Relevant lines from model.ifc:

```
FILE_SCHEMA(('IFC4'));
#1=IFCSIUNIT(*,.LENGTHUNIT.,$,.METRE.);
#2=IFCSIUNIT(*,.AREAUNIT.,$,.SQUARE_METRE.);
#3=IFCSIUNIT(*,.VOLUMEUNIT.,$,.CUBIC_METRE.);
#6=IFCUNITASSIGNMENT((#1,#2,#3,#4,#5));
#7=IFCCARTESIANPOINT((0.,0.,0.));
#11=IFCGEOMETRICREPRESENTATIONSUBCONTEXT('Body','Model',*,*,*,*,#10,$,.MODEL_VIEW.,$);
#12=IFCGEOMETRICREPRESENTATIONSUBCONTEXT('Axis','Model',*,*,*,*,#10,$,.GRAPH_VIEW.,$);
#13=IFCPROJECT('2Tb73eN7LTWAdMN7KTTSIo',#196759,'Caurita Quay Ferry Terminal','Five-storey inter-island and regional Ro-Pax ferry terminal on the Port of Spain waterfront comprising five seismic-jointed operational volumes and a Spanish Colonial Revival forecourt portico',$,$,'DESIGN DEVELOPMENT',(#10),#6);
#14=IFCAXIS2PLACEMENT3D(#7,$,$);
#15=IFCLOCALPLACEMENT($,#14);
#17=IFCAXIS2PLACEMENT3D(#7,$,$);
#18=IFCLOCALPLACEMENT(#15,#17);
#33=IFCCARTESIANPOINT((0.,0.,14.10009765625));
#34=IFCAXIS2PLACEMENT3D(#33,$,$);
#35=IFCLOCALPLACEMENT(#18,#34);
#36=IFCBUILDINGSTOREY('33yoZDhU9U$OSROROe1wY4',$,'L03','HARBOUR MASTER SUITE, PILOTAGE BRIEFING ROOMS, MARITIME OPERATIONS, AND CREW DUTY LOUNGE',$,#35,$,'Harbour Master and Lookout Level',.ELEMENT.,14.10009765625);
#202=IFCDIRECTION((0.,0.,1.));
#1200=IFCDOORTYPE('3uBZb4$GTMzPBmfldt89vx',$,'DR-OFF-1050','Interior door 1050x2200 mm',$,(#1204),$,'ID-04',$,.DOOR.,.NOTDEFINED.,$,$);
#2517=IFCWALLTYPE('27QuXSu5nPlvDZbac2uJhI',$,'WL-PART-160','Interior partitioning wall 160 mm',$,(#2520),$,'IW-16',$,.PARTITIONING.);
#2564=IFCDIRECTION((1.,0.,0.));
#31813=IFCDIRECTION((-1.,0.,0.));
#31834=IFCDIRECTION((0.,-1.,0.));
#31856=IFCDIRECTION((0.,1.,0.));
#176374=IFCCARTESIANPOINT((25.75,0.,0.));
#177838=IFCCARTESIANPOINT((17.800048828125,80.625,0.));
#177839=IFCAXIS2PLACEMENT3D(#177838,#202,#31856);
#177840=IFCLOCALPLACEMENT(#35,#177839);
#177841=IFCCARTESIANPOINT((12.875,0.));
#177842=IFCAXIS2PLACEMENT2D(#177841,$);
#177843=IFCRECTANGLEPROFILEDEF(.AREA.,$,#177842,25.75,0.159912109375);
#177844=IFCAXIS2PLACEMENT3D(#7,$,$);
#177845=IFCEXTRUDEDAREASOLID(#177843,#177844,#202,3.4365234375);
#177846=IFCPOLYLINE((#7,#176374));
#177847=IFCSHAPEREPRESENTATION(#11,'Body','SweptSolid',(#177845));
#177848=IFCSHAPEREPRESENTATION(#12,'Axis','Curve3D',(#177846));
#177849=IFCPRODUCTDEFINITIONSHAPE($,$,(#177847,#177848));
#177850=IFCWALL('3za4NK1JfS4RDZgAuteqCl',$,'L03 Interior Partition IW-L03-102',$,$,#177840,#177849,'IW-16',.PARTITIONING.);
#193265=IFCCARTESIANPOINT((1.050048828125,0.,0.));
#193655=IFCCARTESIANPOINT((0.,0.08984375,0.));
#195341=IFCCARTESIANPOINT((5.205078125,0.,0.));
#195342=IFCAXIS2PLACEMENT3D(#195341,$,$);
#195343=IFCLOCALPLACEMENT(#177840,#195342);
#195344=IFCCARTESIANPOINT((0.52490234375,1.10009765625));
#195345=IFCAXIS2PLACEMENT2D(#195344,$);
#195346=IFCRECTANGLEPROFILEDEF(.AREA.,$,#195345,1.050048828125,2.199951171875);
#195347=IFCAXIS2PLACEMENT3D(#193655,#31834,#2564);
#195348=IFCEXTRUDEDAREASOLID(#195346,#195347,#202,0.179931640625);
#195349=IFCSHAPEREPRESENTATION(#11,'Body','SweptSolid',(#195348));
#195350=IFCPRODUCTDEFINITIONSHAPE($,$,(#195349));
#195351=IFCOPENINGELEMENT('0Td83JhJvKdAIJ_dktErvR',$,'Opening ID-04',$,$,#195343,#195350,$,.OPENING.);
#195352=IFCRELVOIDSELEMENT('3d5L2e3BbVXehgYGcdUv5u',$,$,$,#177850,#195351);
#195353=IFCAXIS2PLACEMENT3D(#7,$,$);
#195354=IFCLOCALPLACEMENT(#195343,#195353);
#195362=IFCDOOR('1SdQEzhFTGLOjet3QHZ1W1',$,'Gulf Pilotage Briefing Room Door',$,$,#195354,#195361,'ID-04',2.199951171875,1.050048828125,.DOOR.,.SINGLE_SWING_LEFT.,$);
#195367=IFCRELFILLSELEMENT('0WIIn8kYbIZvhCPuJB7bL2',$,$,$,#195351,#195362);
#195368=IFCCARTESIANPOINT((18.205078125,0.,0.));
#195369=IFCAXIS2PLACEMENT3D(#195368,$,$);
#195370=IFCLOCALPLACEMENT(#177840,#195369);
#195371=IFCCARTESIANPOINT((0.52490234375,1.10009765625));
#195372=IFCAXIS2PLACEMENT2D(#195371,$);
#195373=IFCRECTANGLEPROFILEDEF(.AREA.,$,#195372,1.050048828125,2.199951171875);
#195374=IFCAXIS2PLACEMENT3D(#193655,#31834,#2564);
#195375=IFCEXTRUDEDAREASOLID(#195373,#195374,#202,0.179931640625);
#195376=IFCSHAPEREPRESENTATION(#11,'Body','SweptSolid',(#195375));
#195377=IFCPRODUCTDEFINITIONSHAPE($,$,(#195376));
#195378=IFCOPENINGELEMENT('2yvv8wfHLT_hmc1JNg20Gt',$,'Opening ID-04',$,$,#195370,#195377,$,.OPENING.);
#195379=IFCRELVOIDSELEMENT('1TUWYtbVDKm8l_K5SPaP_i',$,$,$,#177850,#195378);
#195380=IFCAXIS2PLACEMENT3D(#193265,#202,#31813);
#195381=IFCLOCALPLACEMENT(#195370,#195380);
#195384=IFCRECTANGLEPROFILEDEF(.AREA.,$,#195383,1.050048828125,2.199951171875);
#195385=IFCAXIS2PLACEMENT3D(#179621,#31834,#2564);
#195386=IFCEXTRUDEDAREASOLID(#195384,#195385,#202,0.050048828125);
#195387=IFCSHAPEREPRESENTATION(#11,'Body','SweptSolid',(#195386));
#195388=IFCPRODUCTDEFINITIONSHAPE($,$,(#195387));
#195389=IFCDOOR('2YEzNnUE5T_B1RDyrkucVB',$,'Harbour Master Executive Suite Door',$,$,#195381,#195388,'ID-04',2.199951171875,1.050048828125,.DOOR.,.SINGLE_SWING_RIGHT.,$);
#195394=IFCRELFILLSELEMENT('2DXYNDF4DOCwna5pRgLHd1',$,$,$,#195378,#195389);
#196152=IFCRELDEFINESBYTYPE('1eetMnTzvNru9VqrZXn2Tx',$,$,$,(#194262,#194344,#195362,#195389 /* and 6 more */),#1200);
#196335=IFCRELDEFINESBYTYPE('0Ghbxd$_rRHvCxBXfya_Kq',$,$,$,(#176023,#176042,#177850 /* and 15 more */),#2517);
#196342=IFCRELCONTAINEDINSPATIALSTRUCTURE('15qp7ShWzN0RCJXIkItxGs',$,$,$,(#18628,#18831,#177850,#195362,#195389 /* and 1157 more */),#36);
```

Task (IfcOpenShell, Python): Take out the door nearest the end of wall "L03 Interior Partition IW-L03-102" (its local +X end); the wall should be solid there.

```python
import ifcopenshell
import ifcopenshell.api.feature
import ifcopenshell.api.root
import ifcopenshell.geom
import ifcopenshell.util.shape

model = ifcopenshell.open("model.ifc")
settings = ifcopenshell.geom.settings()


def volume(element):
    """Net volume in cubic metres, openings subtracted."""
    shape = ifcopenshell.geom.create_shape(settings, element)
    return ifcopenshell.util.shape.get_volume(shape.geometry)


door = model.by_id(195389)
opening = door.FillsVoids[0].RelatingOpeningElement
wall = opening.VoidsElements[0].RelatingBuildingElement
before = volume(wall)

ifcopenshell.api.root.remove_product(model, product=door)
ifcopenshell.api.feature.remove_feature(model, feature=opening)

after = volume(wall)

print(f"wall volume {before:.3f} -> {after:.3f} m3")

model.write("model_rev.ifc")
```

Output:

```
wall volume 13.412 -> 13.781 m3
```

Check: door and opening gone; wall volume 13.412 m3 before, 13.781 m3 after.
